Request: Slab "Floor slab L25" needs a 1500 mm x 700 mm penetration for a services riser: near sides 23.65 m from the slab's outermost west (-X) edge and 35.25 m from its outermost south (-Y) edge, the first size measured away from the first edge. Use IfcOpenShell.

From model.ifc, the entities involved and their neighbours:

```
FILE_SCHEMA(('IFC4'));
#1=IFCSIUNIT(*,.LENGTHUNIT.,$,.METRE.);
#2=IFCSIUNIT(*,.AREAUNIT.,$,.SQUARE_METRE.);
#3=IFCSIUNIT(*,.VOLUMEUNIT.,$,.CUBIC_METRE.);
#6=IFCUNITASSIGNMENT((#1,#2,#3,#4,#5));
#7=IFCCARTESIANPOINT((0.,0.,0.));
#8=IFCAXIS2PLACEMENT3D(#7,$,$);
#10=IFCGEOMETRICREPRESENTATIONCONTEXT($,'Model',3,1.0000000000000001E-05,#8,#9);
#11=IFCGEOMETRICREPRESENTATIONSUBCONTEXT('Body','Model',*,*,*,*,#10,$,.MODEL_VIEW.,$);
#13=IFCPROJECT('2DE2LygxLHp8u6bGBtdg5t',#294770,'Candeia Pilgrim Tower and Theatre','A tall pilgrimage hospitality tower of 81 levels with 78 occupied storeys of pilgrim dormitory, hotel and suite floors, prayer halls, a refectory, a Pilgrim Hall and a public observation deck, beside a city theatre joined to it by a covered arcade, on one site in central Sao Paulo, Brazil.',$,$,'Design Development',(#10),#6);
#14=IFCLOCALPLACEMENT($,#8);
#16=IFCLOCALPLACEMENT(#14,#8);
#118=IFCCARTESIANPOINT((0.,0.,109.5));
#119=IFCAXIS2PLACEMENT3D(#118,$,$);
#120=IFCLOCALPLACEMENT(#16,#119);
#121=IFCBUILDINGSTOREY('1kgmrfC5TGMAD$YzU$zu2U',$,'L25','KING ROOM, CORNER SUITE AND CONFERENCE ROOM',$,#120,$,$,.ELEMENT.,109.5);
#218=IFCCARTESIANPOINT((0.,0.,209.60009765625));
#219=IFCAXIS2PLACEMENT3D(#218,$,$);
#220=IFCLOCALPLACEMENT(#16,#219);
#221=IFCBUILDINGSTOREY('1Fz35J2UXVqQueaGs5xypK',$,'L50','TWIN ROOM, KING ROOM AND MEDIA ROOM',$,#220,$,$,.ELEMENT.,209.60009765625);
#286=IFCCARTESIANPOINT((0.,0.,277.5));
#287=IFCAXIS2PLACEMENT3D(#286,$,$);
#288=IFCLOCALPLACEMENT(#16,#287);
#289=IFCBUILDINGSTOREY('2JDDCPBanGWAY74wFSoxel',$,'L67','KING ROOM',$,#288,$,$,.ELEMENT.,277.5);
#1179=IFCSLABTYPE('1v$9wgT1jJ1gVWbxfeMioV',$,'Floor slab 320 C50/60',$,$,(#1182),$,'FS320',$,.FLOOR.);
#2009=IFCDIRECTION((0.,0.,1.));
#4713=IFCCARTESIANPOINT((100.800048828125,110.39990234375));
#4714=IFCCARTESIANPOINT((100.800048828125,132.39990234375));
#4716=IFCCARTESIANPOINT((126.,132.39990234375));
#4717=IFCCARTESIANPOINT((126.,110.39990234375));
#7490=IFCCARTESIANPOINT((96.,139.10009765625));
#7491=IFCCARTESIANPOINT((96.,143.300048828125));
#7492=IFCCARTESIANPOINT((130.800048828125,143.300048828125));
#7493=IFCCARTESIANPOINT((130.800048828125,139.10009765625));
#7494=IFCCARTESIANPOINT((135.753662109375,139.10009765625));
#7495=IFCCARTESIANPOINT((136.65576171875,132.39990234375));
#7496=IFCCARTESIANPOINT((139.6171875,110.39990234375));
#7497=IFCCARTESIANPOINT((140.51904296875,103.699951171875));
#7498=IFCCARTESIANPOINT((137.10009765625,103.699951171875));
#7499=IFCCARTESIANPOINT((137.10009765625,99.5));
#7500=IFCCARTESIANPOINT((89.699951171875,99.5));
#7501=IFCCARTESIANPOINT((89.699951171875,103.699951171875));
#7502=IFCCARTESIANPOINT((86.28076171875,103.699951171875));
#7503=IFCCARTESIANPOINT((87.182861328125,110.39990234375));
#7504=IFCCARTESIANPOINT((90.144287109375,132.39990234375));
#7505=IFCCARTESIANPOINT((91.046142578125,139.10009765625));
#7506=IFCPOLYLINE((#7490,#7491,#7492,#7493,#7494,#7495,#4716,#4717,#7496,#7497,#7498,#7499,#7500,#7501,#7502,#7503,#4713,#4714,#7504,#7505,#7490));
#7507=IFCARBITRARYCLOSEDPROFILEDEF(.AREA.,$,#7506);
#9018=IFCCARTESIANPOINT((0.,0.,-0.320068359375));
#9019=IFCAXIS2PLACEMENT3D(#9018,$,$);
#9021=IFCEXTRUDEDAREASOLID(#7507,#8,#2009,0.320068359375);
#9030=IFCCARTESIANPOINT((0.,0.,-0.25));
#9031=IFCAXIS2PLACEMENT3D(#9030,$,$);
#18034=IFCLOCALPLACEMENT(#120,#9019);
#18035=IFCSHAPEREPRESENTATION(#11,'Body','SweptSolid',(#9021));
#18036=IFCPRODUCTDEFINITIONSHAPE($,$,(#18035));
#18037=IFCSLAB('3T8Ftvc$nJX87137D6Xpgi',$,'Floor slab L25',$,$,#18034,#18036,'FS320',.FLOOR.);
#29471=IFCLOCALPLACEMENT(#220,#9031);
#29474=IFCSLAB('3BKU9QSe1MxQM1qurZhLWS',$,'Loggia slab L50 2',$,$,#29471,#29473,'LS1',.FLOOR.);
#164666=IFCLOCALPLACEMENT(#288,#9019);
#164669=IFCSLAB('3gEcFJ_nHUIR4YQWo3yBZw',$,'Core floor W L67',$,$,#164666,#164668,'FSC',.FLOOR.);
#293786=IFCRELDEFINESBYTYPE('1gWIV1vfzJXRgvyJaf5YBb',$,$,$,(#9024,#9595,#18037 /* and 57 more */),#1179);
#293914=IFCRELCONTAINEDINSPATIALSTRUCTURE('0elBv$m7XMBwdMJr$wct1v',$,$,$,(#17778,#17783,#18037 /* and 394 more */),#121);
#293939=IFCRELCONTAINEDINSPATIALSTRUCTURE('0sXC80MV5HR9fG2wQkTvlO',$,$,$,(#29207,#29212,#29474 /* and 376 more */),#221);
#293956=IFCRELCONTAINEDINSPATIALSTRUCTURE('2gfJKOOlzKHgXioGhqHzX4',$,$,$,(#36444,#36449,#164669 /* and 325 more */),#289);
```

```python
import numpy as np
import ifcopenshell
import ifcopenshell.api.feature
import ifcopenshell.api.geometry
import ifcopenshell.api.root
import ifcopenshell.geom
import ifcopenshell.util.placement
import ifcopenshell.util.representation
import ifcopenshell.util.shape
import ifcopenshell.util.unit

model = ifcopenshell.open("model.ifc")
unit_scale = ifcopenshell.util.unit.calculate_unit_scale(model)
settings = ifcopenshell.geom.settings()


def volume(element):
    """Net volume in cubic metres, openings subtracted."""
    shape = ifcopenshell.geom.create_shape(settings, element)
    return ifcopenshell.util.shape.get_volume(shape.geometry)


slab = model.by_id(18037)
before = volume(slab)

# Extent in the slab's own axes, in metres. The edges named are its -X and -Y sides.
slab_shape = ifcopenshell.geom.create_shape(settings, slab)
vertices = ifcopenshell.util.shape.get_vertices(slab_shape.geometry)
x_min, y_min, bottom = vertices.min(axis=0)
top = vertices[:, 2].max()

opening = ifcopenshell.api.root.create_entity(model, ifc_class="IfcOpeningElement", name="Services riser opening", predefined_type="OPENING")
context = ifcopenshell.util.representation.get_context(model, "Model", "Body", "MODEL_VIEW")
width, depth = 1.5, 0.7
outline = [(0.0, 0.0), (width, 0.0), (width, depth), (0.0, depth), (0.0, 0.0)]
# Overshoot both faces by 50 mm so the cut is clean.
shape = ifcopenshell.api.geometry.add_slab_representation(
    model, context=context, depth=top - bottom + 0.1, polyline=outline
)
ifcopenshell.api.geometry.assign_representation(model, product=opening, representation=shape)

matrix = ifcopenshell.util.placement.get_local_placement(slab.ObjectPlacement)
matrix[:, 3] = matrix @ np.append(np.array([x_min + 23.65, y_min + 35.25, bottom - 0.05]) / unit_scale, 1.0)
ifcopenshell.api.geometry.edit_object_placement(model, product=opening, matrix=matrix, is_si=False)
ifcopenshell.api.feature.add_feature(model, feature=opening, element=slab)

after = volume(slab)

print(f"slab volume {before:.3f} -> {after:.3f} m3")

model.write("model_edited.ifc")
```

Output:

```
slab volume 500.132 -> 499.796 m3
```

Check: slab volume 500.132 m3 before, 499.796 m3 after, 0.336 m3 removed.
